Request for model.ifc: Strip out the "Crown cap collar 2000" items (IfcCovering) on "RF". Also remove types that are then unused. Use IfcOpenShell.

First a look at what the model holds.

```python
import ifcopenshell
import ifcopenshell.util.element

model = ifcopenshell.open("model.ifc")
print(model.schema)
storey = next(s for s in model.by_type("IfcBuildingStorey") if s.Name == "RF")
coverings = [e for e in ifcopenshell.util.element.get_decomposition(storey) if e.is_a("IfcCovering")]
seen = {}
for e in coverings:
    element_type = ifcopenshell.util.element.get_type(e)
    name = element_type.Name if element_type not in (None, e) else None
    seen[name] = seen.get(name, 0) + 1
for name, count in sorted(seen.items(), key=str):
    print(count, "x", name)
```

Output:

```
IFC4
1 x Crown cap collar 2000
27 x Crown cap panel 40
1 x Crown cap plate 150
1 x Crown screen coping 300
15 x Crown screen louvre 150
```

```python
import ifcopenshell
import ifcopenshell.api.root
import ifcopenshell.util.element

model = ifcopenshell.open("model.ifc")

storey = next(s for s in model.by_type("IfcBuildingStorey") if s.Name == "RF")
coverings = [e for e in ifcopenshell.util.element.get_decomposition(storey) if e.is_a("IfcCovering")]
targets = [e for e in coverings if (t := ifcopenshell.util.element.get_type(e)) not in (None, e) and t.Name == "Crown cap collar 2000"]
types = {ifcopenshell.util.element.get_type(e) for e in targets} - {None, *targets}

for e in targets:
    ifcopenshell.api.root.remove_product(model, product=e)
print(len(targets), "removed")

unused = [t for t in types if not ifcopenshell.util.element.get_types(t)]
for t in unused:
    ifcopenshell.api.root.remove_product(model, product=t)
print(len(unused), "unused types removed")

model.write("model_v2.ifc")
```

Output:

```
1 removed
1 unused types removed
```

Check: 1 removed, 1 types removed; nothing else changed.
